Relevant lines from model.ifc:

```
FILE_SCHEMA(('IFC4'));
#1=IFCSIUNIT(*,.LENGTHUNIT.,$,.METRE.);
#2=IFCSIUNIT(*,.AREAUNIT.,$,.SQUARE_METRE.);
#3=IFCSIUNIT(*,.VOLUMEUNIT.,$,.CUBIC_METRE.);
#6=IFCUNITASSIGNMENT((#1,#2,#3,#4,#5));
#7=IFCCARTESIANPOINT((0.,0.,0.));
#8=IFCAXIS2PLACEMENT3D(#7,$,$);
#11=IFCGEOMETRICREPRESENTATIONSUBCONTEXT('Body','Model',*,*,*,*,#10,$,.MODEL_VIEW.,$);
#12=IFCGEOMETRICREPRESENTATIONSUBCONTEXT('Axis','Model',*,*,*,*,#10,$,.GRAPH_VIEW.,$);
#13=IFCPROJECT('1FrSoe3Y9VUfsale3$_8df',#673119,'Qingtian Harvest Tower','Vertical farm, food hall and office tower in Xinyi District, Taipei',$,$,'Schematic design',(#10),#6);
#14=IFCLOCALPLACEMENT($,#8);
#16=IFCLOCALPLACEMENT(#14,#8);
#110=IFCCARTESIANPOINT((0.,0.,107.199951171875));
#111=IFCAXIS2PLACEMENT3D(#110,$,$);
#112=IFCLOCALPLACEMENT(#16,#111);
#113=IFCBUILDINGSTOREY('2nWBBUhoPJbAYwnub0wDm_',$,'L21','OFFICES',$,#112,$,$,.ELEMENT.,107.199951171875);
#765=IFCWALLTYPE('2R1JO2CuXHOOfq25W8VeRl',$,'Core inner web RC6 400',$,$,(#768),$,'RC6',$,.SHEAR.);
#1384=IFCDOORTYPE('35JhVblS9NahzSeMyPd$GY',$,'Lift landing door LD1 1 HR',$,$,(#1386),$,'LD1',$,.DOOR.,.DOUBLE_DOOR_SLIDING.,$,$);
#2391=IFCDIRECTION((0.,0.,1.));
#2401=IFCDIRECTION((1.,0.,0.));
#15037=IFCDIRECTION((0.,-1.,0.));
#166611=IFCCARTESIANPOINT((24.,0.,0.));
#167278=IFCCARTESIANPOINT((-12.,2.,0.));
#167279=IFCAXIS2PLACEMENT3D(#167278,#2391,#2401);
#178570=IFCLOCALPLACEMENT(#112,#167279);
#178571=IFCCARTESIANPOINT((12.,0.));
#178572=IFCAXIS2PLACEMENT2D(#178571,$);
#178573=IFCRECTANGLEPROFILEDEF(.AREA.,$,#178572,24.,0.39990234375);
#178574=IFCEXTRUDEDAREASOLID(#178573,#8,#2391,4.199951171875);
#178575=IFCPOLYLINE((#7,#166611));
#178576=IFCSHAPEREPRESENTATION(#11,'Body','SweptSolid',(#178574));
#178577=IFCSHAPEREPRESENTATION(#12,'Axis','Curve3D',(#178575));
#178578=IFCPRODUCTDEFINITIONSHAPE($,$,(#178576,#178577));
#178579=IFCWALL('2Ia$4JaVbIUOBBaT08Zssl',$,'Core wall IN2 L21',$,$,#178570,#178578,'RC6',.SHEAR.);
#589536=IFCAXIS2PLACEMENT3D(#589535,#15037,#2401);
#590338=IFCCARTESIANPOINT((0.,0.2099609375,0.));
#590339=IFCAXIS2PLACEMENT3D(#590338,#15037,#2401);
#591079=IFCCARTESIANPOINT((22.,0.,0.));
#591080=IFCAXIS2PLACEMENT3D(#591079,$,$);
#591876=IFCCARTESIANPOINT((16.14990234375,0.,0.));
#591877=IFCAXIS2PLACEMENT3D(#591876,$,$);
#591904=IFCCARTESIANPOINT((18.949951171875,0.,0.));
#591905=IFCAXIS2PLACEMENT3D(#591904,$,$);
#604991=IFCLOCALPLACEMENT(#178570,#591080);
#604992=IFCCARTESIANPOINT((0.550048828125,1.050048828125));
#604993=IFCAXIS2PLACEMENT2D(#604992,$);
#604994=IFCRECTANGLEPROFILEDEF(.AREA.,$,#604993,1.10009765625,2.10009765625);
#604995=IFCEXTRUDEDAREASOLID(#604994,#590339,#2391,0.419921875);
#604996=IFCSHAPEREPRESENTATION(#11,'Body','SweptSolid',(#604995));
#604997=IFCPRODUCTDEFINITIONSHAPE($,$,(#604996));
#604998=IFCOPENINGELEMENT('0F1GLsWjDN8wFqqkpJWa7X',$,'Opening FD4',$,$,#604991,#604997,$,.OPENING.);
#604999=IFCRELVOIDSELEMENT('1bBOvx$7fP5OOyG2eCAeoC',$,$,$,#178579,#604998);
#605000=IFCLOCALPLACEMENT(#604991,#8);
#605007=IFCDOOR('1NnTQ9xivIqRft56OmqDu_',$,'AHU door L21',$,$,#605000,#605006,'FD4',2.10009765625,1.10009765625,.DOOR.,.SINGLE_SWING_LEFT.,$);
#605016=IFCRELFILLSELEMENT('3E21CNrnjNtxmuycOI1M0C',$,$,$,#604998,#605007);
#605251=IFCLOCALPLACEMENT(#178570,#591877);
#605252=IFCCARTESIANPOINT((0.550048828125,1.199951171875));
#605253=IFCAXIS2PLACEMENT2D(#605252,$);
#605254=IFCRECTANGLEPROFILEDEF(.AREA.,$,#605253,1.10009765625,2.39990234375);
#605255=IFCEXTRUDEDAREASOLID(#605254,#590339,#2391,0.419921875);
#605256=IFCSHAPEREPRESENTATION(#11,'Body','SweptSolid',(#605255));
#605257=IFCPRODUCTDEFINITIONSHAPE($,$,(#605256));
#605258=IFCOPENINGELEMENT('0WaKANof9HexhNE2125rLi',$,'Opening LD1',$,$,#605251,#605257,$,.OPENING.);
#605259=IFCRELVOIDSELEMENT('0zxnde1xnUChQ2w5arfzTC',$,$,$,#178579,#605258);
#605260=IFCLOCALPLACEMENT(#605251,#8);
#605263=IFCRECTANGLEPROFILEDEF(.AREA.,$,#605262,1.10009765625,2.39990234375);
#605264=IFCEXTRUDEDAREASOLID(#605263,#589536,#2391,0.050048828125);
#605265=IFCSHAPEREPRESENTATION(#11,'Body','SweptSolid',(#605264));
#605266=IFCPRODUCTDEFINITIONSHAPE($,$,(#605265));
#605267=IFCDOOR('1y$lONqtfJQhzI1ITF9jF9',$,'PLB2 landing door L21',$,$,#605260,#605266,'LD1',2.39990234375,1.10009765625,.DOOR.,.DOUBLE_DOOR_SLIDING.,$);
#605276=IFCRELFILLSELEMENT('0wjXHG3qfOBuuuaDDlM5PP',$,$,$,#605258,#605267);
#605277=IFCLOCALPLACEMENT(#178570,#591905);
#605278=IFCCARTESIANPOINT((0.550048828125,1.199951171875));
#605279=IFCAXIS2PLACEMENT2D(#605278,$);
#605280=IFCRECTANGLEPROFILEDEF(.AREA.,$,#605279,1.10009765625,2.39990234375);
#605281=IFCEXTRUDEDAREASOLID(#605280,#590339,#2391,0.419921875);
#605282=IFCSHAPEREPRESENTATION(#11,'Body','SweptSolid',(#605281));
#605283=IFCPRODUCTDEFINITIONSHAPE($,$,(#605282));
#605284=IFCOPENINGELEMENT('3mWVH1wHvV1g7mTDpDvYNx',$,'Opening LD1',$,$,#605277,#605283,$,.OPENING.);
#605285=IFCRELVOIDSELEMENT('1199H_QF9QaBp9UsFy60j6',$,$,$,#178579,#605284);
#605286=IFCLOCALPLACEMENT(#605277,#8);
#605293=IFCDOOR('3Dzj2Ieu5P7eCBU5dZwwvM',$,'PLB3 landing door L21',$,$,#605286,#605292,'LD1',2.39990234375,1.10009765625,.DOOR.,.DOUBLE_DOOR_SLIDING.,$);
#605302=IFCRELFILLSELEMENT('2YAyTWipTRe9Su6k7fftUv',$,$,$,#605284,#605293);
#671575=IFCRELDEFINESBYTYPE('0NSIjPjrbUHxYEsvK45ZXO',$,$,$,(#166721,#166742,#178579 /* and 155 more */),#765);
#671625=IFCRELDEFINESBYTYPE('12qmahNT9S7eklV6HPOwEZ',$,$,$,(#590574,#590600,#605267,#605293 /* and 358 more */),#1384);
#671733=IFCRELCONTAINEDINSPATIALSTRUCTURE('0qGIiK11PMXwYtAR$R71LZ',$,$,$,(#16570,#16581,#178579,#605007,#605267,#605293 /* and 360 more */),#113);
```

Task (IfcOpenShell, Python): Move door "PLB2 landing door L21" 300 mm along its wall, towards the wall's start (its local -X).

```python
import ifcopenshell
import ifcopenshell.api.geometry
import ifcopenshell.util.placement
import ifcopenshell.util.unit

model = ifcopenshell.open("model.ifc")
unit_scale = ifcopenshell.util.unit.calculate_unit_scale(model)

door = model.by_id(605267)
opening = door.FillsVoids[0].RelatingOpeningElement
wall = opening.VoidsElements[0].RelatingBuildingElement

wall_matrix = ifcopenshell.util.placement.get_local_placement(wall.ObjectPlacement)
shift = wall_matrix[:3, 0] * -0.3 / unit_scale
before = ifcopenshell.util.placement.get_local_placement(door.ObjectPlacement)[:3, 3].copy()

# The door is placed relative to its opening, so it follows when the opening moves.
matrix = ifcopenshell.util.placement.get_local_placement(opening.ObjectPlacement)
matrix[:3, 3] += shift
ifcopenshell.api.geometry.edit_object_placement(
    model, product=opening, matrix=matrix, is_si=False, should_transform_children=True
)

after = ifcopenshell.util.placement.get_local_placement(door.ObjectPlacement)[:3, 3]
print("door moved by", (after - before).round(3) + 0.0)

model.write("model_edited.ifc")
```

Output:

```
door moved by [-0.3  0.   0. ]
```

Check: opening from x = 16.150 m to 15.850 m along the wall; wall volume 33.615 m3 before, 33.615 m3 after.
